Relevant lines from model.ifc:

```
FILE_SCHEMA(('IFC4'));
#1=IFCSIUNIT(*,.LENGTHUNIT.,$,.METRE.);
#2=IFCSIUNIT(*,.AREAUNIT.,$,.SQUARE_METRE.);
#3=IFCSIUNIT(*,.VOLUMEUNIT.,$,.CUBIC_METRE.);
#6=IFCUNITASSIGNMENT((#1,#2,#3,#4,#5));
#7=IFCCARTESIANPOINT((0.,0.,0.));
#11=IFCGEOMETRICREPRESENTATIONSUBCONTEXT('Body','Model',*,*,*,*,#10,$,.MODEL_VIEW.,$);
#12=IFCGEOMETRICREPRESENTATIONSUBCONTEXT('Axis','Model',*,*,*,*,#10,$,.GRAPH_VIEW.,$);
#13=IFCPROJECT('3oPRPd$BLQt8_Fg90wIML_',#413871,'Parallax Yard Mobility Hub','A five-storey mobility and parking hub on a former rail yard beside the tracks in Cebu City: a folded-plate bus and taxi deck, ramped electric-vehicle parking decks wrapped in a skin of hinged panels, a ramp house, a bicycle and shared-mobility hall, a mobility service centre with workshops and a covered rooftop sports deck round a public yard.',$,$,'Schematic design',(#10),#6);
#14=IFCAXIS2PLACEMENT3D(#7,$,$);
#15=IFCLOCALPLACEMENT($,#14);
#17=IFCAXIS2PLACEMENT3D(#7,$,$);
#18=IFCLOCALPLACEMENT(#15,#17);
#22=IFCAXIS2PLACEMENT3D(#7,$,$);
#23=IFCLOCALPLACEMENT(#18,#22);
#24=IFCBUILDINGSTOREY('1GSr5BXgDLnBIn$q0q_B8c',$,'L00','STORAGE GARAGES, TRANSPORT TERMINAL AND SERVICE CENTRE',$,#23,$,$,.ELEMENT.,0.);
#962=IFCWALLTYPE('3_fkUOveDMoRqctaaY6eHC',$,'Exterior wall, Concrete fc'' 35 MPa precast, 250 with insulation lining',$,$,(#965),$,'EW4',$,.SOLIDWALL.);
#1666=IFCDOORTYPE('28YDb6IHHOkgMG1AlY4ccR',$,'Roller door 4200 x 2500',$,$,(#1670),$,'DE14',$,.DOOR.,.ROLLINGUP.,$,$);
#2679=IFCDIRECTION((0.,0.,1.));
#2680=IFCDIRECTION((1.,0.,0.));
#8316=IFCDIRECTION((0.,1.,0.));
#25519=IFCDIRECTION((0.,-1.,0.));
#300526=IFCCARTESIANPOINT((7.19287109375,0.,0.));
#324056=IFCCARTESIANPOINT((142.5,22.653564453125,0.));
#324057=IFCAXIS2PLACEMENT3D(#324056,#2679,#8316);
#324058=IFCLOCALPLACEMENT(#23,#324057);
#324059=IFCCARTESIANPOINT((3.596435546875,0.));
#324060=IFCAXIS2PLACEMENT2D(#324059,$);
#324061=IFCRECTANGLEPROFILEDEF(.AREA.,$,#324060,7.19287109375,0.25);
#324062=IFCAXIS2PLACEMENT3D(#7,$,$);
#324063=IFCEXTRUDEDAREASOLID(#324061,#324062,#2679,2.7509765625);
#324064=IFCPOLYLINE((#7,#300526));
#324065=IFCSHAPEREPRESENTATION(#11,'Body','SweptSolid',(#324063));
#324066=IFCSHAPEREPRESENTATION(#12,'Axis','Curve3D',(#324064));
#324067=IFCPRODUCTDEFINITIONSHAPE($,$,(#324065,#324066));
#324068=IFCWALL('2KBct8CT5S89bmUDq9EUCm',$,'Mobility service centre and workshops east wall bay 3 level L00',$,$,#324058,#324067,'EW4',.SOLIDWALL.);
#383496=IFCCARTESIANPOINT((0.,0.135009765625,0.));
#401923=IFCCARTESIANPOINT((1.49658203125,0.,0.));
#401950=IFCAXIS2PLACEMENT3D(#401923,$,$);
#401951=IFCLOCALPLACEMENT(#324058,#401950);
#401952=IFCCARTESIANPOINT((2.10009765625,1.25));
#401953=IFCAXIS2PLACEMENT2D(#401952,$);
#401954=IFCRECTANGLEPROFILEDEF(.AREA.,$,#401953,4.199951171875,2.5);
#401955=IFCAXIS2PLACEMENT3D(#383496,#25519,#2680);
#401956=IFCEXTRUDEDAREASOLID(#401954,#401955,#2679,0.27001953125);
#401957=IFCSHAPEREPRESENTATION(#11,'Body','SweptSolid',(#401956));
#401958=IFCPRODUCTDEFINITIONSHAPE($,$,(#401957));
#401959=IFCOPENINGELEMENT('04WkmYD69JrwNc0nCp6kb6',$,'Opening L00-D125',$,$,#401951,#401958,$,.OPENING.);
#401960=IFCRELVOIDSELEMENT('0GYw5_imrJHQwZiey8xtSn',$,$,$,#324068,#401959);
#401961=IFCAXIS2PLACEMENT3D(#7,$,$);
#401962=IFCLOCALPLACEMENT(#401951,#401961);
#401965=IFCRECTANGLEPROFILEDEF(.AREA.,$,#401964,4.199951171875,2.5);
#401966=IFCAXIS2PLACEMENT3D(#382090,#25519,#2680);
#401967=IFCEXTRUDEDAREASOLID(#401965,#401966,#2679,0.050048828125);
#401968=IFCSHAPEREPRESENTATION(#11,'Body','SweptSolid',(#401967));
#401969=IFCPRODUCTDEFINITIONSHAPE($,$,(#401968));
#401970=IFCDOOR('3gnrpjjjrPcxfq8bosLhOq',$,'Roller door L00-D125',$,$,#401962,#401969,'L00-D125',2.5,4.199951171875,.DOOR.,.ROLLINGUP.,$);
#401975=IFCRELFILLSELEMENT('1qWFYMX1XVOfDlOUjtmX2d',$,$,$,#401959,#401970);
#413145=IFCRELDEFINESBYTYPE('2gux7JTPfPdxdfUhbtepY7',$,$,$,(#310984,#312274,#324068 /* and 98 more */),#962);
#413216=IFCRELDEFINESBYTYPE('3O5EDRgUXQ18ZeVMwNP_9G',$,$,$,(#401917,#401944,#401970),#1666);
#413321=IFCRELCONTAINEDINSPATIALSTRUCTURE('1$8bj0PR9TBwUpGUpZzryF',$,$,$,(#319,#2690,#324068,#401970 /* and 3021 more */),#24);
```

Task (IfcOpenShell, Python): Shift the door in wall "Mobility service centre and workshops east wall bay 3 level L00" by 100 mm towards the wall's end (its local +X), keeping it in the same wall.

```python
import ifcopenshell
import ifcopenshell.api.geometry
import ifcopenshell.util.placement
import ifcopenshell.util.unit

model = ifcopenshell.open("model.ifc")
unit_scale = ifcopenshell.util.unit.calculate_unit_scale(model)

door = model.by_guid("3gnrpjjjrPcxfq8bosLhOq")
opening = door.FillsVoids[0].RelatingOpeningElement
wall = opening.VoidsElements[0].RelatingBuildingElement

wall_matrix = ifcopenshell.util.placement.get_local_placement(wall.ObjectPlacement)
shift = wall_matrix[:3, 0] * 0.1 / unit_scale
before = ifcopenshell.util.placement.get_local_placement(door.ObjectPlacement)[:3, 3].copy()

# The door is placed relative to its opening, so it follows when the opening moves.
matrix = ifcopenshell.util.placement.get_local_placement(opening.ObjectPlacement)
matrix[:3, 3] += shift
ifcopenshell.api.geometry.edit_object_placement(
    model, product=opening, matrix=matrix, is_si=False, should_transform_children=True
)

after = ifcopenshell.util.placement.get_local_placement(door.ObjectPlacement)[:3, 3]
print("door moved by", (after - before).round(3) + 0.0)

model.write("model-out.ifc")
```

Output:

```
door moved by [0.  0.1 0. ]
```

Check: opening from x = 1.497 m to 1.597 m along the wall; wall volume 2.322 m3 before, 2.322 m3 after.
